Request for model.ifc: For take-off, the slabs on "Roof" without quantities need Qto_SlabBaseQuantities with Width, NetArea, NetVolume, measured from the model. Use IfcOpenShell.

First a look at what the model holds.

```python
import ifcopenshell
import ifcopenshell.util.element
import ifcopenshell.util.unit

model = ifcopenshell.open("model.ifc")
print(model.schema)
for unit_type in ("LENGTHUNIT", "AREAUNIT", "VOLUMEUNIT"):
    print(unit_type, ifcopenshell.util.unit.calculate_unit_scale(model, unit_type))
storey = next(s for s in model.by_type("IfcBuildingStorey") if s.Name == "Roof")
slabs = [e for e in ifcopenshell.util.element.get_decomposition(storey) if e.is_a("IfcSlab")]
for e in sorted(slabs, key=lambda e: e.id()):
    print(e.id(), e.is_a(), e.Name, list(ifcopenshell.util.element.get_psets(e, qtos_only=True)), sep=" | ")
```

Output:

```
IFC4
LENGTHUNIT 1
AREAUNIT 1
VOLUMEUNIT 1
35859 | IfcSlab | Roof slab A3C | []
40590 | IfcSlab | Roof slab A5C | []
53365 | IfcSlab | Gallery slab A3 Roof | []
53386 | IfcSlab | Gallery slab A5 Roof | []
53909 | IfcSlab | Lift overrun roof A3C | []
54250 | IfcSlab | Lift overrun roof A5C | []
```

```python
import ifcopenshell
import ifcopenshell.api.pset
import ifcopenshell.geom
import ifcopenshell.util.element
import ifcopenshell.util.shape
import ifcopenshell.util.unit

model = ifcopenshell.open("model.ifc")
unit_scale = ifcopenshell.util.unit.calculate_unit_scale(model)
area_scale = ifcopenshell.util.unit.calculate_unit_scale(model, "AREAUNIT")
volume_scale = ifcopenshell.util.unit.calculate_unit_scale(model, "VOLUMEUNIT")
settings = ifcopenshell.geom.settings()

storey = next(s for s in model.by_type("IfcBuildingStorey") if s.Name == "Roof")
slabs = [e for e in ifcopenshell.util.element.get_decomposition(storey) if e.is_a("IfcSlab")]

for e in sorted(slabs, key=lambda e: e.id()):
    if ifcopenshell.util.element.get_psets(e, qtos_only=True, should_inherit=False):
        continue
    # Geometry comes back in metres, in the element's own axes.
    shape = ifcopenshell.geom.create_shape(settings, e)
    values = {
        "Width": ifcopenshell.util.shape.get_z(shape.geometry) / unit_scale,
        "NetArea": ifcopenshell.util.shape.get_footprint_area(shape.geometry) / area_scale,
        "NetVolume": ifcopenshell.util.shape.get_volume(shape.geometry) / volume_scale,
    }
    qto = ifcopenshell.api.pset.add_qto(model, product=e, name="Qto_SlabBaseQuantities")
    ifcopenshell.api.pset.edit_qto(model, qto=qto, properties=values)
    print(e.id(), {k: round(v, 3) for k, v in values.items()})

model.write("model-out.ifc")
```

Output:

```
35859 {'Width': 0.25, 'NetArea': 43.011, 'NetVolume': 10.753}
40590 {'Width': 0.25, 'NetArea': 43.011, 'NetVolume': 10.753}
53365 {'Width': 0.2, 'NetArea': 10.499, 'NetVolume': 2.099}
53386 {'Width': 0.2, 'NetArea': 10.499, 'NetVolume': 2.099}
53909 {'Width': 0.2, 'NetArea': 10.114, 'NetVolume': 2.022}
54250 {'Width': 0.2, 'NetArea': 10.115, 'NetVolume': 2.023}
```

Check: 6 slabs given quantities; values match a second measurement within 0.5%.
